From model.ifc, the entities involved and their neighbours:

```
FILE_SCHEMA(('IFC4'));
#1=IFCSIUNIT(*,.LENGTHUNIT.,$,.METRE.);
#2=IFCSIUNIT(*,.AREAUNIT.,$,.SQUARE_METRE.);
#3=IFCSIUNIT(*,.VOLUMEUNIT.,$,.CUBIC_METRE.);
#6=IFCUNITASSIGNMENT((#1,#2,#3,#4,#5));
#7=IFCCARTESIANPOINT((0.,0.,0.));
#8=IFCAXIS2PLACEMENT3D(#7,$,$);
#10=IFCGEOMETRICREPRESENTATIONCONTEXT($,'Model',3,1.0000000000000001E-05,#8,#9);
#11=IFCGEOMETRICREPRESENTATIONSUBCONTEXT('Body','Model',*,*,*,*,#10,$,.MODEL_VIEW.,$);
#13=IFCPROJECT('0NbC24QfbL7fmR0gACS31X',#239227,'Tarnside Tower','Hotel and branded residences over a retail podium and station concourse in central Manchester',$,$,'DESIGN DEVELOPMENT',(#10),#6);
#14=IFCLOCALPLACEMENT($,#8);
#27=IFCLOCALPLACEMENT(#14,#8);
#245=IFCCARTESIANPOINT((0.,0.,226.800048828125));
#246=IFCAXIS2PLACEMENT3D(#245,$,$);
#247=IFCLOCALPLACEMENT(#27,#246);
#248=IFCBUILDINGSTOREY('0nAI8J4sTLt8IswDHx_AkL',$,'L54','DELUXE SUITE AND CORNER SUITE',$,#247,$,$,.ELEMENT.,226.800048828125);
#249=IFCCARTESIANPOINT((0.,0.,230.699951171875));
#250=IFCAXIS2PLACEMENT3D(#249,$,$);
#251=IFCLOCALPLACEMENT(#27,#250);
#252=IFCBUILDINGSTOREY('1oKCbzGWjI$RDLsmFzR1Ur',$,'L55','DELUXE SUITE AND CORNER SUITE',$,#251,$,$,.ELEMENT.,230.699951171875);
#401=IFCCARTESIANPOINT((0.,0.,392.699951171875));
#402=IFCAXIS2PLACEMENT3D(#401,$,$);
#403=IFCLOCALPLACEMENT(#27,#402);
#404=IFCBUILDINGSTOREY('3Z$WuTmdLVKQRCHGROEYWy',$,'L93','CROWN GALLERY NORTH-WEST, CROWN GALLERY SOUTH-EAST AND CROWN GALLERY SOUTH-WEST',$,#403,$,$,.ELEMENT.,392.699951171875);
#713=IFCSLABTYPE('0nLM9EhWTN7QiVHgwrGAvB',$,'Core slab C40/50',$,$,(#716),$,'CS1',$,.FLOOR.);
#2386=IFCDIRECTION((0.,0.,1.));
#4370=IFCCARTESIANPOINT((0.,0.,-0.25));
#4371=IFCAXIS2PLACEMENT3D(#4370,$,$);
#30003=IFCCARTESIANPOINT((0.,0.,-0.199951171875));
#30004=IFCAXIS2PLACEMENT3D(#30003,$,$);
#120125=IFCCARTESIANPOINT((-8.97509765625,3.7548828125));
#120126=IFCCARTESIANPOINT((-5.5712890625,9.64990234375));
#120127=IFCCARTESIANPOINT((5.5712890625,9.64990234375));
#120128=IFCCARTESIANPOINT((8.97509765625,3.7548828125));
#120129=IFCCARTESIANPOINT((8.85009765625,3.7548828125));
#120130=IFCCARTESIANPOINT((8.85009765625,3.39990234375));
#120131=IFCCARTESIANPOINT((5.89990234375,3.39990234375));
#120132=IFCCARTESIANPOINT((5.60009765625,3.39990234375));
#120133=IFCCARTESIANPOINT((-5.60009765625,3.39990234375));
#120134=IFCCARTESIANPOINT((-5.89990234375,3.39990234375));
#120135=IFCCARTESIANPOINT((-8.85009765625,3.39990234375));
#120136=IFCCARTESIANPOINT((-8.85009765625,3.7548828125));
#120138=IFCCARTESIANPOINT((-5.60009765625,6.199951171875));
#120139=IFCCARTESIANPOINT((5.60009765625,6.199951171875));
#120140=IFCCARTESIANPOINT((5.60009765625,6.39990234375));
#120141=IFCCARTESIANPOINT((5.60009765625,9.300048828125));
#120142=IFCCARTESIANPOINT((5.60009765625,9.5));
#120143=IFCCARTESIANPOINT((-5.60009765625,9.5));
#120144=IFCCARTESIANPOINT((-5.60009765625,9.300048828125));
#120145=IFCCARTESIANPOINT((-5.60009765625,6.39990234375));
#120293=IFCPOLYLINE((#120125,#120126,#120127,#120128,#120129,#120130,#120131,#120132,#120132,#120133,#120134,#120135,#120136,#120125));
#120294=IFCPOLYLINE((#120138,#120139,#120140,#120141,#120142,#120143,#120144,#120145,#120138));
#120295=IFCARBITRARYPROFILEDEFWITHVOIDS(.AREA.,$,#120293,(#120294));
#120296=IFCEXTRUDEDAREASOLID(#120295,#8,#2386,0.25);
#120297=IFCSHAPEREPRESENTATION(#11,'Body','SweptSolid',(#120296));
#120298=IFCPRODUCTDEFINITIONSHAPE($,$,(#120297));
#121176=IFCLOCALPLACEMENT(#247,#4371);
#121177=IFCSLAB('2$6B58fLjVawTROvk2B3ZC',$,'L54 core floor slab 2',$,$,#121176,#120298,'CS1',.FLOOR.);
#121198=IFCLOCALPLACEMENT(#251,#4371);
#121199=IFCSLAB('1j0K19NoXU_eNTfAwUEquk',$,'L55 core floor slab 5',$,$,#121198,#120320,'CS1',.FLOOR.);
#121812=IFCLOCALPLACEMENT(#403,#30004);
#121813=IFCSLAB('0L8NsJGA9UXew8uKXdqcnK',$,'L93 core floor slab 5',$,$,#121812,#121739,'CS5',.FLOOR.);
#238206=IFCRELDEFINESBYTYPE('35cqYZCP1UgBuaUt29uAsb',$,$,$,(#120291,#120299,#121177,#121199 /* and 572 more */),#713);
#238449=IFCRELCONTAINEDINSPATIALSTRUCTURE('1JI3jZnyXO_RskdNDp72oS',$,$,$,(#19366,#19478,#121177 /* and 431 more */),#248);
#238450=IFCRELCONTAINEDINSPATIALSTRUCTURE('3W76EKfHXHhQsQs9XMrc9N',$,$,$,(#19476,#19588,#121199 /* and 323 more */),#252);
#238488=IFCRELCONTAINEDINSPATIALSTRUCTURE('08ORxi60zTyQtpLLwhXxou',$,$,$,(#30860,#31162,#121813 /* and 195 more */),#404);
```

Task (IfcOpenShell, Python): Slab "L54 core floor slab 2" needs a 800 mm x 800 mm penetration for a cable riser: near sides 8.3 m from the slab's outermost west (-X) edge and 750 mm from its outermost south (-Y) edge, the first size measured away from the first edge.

```python
import numpy as np
import ifcopenshell
import ifcopenshell.api.feature
import ifcopenshell.api.geometry
import ifcopenshell.api.root
import ifcopenshell.geom
import ifcopenshell.util.placement
import ifcopenshell.util.representation
import ifcopenshell.util.shape
import ifcopenshell.util.unit

model = ifcopenshell.open("model.ifc")
unit_scale = ifcopenshell.util.unit.calculate_unit_scale(model)
settings = ifcopenshell.geom.settings()


def volume(element):
    """Net volume in cubic metres, openings subtracted."""
    shape = ifcopenshell.geom.create_shape(settings, element)
    return ifcopenshell.util.shape.get_volume(shape.geometry)


slab = model.by_guid("2$6B58fLjVawTROvk2B3ZC")
before = volume(slab)

# Extent in the slab's own axes, in metres. The edges named are its -X and -Y sides.
slab_shape = ifcopenshell.geom.create_shape(settings, slab)
vertices = ifcopenshell.util.shape.get_vertices(slab_shape.geometry)
x_min, y_min, bottom = vertices.min(axis=0)
top = vertices[:, 2].max()

opening = ifcopenshell.api.root.create_entity(model, ifc_class="IfcOpeningElement", name="Cable riser opening", predefined_type="OPENING")
context = ifcopenshell.util.representation.get_context(model, "Model", "Body", "MODEL_VIEW")
width, depth = 0.8, 0.8
outline = [(0.0, 0.0), (width, 0.0), (width, depth), (0.0, depth), (0.0, 0.0)]
# Overshoot both faces by 50 mm so the cut is clean.
shape = ifcopenshell.api.geometry.add_slab_representation(
    model, context=context, depth=top - bottom + 0.1, polyline=outline
)
ifcopenshell.api.geometry.assign_representation(model, product=opening, representation=shape)

matrix = ifcopenshell.util.placement.get_local_placement(slab.ObjectPlacement)
matrix[:, 3] = matrix @ np.append(np.array([x_min + 8.3, y_min + 0.75, bottom - 0.05]) / unit_scale, 1.0)
ifcopenshell.api.geometry.edit_object_placement(model, product=opening, matrix=matrix, is_si=False)
ifcopenshell.api.feature.add_feature(model, feature=opening, element=slab)

after = volume(slab)

print(f"slab volume {before:.3f} -> {after:.3f} m3")

model.write("model_rev.ifc")
```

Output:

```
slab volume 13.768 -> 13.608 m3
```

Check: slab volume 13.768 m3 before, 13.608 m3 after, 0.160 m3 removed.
